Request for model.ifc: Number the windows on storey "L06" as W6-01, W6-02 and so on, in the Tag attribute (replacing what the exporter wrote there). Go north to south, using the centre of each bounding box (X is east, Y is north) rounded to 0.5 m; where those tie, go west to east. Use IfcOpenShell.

First a look at what the model holds.

```python
import ifcopenshell
import ifcopenshell.util.element
import ifcopenshell.util.placement

model = ifcopenshell.open("model.ifc")
print(model.schema)
storey = next(s for s in model.by_type("IfcBuildingStorey") if s.Name == "L06")
windows = [e for e in ifcopenshell.util.element.get_decomposition(storey) if e.is_a("IfcWindow")]
for e in sorted(windows, key=lambda e: e.id()):
    origin = ifcopenshell.util.placement.get_local_placement(e.ObjectPlacement)[:3, 3]
    print(e.id(), e.Tag, e.Name, origin.round(2) + 0.0, sep=" | ")
```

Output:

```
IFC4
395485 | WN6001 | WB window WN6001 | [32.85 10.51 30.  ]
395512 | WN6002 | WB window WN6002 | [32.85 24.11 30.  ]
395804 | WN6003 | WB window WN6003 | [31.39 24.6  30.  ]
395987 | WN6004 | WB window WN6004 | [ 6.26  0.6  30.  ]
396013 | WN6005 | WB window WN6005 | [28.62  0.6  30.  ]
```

```python
import ifcopenshell
import ifcopenshell.geom
import ifcopenshell.util.element
import ifcopenshell.util.shape

model = ifcopenshell.open("model.ifc")
settings = ifcopenshell.geom.settings()
settings.set("use-world-coords", True)


def centre(element):
    shape = ifcopenshell.geom.create_shape(settings, element)
    return ifcopenshell.util.shape.get_bbox_centroid(shape.geometry)


storey = next(s for s in model.by_type("IfcBuildingStorey") if s.Name == "L06")
windows = [e for e in ifcopenshell.util.element.get_decomposition(storey) if e.is_a("IfcWindow")]

# Insertion points can sit at a corner or the storey origin, so sort by the geometry (in metres).
centres = {e: centre(e) for e in windows}
windows.sort(key=lambda e: (-round(centres[e][1] / 0.5), centres[e][0]))

for i, e in enumerate(windows, start=1):
    number = f"W6-{i:02d}"
    e.Tag = number
    print(e.id(), number)

model.write("model_edited.ifc")
```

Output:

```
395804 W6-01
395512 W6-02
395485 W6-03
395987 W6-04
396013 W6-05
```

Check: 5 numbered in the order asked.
